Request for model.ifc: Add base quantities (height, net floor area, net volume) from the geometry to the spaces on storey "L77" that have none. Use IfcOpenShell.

First a look at what the model holds.

```python
import ifcopenshell
import ifcopenshell.util.element
import ifcopenshell.util.unit

model = ifcopenshell.open("model.ifc")
print(model.schema)
for unit_type in ("LENGTHUNIT", "AREAUNIT", "VOLUMEUNIT"):
    print(unit_type, ifcopenshell.util.unit.calculate_unit_scale(model, unit_type))
storey = next(s for s in model.by_type("IfcBuildingStorey") if s.Name == "L77")
spaces = [e for e in ifcopenshell.util.element.get_decomposition(storey) if e.is_a("IfcSpace")]
for e in sorted(spaces, key=lambda e: e.id()):
    print(e.id(), e.is_a(), e.Name, list(ifcopenshell.util.element.get_psets(e, qtos_only=True)), sep=" | ")
```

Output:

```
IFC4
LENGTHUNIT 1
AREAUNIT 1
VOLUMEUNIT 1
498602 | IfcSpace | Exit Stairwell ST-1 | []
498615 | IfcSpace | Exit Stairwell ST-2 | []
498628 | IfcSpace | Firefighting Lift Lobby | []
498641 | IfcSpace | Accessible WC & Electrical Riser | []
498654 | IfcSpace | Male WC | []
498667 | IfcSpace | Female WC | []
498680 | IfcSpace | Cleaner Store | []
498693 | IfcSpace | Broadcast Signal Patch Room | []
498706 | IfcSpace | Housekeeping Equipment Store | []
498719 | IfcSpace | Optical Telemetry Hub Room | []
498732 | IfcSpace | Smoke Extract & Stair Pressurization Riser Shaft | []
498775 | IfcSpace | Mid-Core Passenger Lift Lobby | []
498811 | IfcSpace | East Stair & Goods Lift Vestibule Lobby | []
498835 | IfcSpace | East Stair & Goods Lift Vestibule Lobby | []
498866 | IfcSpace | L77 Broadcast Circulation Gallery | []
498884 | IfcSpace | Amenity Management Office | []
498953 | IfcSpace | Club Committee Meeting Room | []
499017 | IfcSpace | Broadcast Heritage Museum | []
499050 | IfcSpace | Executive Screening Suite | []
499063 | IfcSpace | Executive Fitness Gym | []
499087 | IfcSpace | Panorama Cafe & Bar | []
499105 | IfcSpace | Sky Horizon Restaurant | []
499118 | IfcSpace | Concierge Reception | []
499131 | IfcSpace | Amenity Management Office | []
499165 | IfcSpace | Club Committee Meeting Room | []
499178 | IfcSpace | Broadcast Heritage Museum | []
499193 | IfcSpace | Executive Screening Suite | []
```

```python
import ifcopenshell
import ifcopenshell.api.pset
import ifcopenshell.geom
import ifcopenshell.util.element
import ifcopenshell.util.shape
import ifcopenshell.util.unit

model = ifcopenshell.open("model.ifc")
unit_scale = ifcopenshell.util.unit.calculate_unit_scale(model)
area_scale = ifcopenshell.util.unit.calculate_unit_scale(model, "AREAUNIT")
volume_scale = ifcopenshell.util.unit.calculate_unit_scale(model, "VOLUMEUNIT")
settings = ifcopenshell.geom.settings()

storey = next(s for s in model.by_type("IfcBuildingStorey") if s.Name == "L77")
spaces = [e for e in ifcopenshell.util.element.get_decomposition(storey) if e.is_a("IfcSpace")]

for e in sorted(spaces, key=lambda e: e.id()):
    if ifcopenshell.util.element.get_psets(e, qtos_only=True, should_inherit=False):
        continue
    # Geometry comes back in metres, in the element's own axes.
    shape = ifcopenshell.geom.create_shape(settings, e)
    values = {
        "Height": ifcopenshell.util.shape.get_z(shape.geometry) / unit_scale,
        "NetFloorArea": ifcopenshell.util.shape.get_footprint_area(shape.geometry) / area_scale,
        "NetVolume": ifcopenshell.util.shape.get_volume(shape.geometry) / volume_scale,
    }
    qto = ifcopenshell.api.pset.add_qto(model, product=e, name="Qto_SpaceBaseQuantities")
    ifcopenshell.api.pset.edit_qto(model, qto=qto, properties=values)
    print(e.id(), {k: round(v, 3) for k, v in values.items()})

model.write("model_v2.ifc")
```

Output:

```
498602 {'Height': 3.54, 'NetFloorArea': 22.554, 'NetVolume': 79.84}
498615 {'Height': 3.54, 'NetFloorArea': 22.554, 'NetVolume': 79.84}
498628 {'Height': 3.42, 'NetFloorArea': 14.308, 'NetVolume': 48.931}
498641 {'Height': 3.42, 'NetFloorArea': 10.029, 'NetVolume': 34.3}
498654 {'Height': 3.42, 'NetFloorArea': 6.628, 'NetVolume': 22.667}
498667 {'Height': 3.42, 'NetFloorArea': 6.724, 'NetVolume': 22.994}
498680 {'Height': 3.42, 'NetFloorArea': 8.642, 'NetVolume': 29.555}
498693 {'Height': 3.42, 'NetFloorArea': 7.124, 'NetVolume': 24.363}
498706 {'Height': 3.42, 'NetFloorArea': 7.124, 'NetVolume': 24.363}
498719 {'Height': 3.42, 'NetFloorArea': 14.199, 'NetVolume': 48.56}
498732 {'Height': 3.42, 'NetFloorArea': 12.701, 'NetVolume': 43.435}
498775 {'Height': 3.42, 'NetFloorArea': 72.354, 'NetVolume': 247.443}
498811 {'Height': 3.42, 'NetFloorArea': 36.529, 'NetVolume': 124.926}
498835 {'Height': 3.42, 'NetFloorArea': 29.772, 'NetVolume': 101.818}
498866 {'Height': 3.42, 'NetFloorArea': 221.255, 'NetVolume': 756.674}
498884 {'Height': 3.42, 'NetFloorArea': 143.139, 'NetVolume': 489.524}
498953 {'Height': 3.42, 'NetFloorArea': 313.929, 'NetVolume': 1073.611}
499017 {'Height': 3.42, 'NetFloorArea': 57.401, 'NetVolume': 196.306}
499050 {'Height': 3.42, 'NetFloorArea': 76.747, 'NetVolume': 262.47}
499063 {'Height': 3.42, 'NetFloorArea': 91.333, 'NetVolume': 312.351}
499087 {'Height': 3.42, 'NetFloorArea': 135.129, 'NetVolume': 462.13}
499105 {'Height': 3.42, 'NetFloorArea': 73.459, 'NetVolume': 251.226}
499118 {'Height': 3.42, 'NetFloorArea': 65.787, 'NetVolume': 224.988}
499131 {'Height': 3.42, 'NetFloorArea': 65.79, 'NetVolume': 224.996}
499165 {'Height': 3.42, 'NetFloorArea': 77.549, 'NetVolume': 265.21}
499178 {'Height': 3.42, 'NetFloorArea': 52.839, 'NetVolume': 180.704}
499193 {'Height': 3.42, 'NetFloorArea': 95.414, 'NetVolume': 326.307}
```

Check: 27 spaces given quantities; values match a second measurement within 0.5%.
